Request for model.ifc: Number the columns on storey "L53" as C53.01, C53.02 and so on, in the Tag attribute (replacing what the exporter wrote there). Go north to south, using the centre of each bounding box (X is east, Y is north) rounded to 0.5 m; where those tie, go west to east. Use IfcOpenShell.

First a look at what the model holds.

```python
import ifcopenshell
import ifcopenshell.util.element
import ifcopenshell.util.placement

model = ifcopenshell.open("model.ifc")
print(model.schema)
storey = next(s for s in model.by_type("IfcBuildingStorey") if s.Name == "L53")
columns = [e for e in ifcopenshell.util.element.get_decomposition(storey) if e.is_a("IfcColumn")]
for e in sorted(columns, key=lambda e: e.id()):
    origin = ifcopenshell.util.placement.get_local_placement(e.ObjectPlacement)[:3, 3]
    print(e.id(), e.Tag, e.Name, origin.round(2) + 0.0, sep=" | ")
```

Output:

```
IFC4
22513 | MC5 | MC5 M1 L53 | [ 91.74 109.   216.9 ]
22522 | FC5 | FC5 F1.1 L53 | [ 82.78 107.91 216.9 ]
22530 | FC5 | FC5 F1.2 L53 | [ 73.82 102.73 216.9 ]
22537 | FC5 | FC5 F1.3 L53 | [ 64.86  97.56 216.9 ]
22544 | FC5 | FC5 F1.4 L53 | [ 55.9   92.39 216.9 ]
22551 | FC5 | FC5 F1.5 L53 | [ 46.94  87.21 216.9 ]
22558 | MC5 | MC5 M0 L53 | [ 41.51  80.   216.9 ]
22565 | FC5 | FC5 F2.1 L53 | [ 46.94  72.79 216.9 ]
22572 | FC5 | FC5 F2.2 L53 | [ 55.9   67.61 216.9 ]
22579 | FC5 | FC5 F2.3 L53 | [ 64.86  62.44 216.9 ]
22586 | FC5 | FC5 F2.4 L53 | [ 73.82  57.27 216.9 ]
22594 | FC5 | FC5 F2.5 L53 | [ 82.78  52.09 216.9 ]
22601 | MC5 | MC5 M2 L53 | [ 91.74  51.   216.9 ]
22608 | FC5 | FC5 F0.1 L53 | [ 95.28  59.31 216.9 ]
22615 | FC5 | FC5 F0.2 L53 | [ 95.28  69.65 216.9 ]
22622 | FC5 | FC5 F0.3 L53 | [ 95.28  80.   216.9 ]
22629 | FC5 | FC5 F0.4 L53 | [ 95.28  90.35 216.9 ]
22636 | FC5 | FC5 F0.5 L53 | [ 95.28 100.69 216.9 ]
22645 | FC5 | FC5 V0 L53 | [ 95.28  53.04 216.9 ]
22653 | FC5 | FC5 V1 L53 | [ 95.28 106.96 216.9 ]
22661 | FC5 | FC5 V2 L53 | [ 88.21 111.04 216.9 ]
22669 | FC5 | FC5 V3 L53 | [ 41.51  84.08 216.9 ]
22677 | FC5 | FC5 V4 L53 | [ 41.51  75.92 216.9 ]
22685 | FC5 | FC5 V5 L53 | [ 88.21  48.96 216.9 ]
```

```python
import ifcopenshell
import ifcopenshell.geom
import ifcopenshell.util.element
import ifcopenshell.util.shape

model = ifcopenshell.open("model.ifc")
settings = ifcopenshell.geom.settings()
settings.set("use-world-coords", True)


def centre(element):
    shape = ifcopenshell.geom.create_shape(settings, element)
    return ifcopenshell.util.shape.get_bbox_centroid(shape.geometry)


storey = next(s for s in model.by_type("IfcBuildingStorey") if s.Name == "L53")
columns = [e for e in ifcopenshell.util.element.get_decomposition(storey) if e.is_a("IfcColumn")]

# Insertion points can sit at a corner or the storey origin, so sort by the geometry (in metres).
centres = {e: centre(e) for e in columns}
columns.sort(key=lambda e: (-round(centres[e][1] / 0.5), centres[e][0]))

for i, e in enumerate(columns, start=1):
    number = f"C53.{i:02d}"
    e.Tag = number
    print(e.id(), number)

model.write("model_v2.ifc")
```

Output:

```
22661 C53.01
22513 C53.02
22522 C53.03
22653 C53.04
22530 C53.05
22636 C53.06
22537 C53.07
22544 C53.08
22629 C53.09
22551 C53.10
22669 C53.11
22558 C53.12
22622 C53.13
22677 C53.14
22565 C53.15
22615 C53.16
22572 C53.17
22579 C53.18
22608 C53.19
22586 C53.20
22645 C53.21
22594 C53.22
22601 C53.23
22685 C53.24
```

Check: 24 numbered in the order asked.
